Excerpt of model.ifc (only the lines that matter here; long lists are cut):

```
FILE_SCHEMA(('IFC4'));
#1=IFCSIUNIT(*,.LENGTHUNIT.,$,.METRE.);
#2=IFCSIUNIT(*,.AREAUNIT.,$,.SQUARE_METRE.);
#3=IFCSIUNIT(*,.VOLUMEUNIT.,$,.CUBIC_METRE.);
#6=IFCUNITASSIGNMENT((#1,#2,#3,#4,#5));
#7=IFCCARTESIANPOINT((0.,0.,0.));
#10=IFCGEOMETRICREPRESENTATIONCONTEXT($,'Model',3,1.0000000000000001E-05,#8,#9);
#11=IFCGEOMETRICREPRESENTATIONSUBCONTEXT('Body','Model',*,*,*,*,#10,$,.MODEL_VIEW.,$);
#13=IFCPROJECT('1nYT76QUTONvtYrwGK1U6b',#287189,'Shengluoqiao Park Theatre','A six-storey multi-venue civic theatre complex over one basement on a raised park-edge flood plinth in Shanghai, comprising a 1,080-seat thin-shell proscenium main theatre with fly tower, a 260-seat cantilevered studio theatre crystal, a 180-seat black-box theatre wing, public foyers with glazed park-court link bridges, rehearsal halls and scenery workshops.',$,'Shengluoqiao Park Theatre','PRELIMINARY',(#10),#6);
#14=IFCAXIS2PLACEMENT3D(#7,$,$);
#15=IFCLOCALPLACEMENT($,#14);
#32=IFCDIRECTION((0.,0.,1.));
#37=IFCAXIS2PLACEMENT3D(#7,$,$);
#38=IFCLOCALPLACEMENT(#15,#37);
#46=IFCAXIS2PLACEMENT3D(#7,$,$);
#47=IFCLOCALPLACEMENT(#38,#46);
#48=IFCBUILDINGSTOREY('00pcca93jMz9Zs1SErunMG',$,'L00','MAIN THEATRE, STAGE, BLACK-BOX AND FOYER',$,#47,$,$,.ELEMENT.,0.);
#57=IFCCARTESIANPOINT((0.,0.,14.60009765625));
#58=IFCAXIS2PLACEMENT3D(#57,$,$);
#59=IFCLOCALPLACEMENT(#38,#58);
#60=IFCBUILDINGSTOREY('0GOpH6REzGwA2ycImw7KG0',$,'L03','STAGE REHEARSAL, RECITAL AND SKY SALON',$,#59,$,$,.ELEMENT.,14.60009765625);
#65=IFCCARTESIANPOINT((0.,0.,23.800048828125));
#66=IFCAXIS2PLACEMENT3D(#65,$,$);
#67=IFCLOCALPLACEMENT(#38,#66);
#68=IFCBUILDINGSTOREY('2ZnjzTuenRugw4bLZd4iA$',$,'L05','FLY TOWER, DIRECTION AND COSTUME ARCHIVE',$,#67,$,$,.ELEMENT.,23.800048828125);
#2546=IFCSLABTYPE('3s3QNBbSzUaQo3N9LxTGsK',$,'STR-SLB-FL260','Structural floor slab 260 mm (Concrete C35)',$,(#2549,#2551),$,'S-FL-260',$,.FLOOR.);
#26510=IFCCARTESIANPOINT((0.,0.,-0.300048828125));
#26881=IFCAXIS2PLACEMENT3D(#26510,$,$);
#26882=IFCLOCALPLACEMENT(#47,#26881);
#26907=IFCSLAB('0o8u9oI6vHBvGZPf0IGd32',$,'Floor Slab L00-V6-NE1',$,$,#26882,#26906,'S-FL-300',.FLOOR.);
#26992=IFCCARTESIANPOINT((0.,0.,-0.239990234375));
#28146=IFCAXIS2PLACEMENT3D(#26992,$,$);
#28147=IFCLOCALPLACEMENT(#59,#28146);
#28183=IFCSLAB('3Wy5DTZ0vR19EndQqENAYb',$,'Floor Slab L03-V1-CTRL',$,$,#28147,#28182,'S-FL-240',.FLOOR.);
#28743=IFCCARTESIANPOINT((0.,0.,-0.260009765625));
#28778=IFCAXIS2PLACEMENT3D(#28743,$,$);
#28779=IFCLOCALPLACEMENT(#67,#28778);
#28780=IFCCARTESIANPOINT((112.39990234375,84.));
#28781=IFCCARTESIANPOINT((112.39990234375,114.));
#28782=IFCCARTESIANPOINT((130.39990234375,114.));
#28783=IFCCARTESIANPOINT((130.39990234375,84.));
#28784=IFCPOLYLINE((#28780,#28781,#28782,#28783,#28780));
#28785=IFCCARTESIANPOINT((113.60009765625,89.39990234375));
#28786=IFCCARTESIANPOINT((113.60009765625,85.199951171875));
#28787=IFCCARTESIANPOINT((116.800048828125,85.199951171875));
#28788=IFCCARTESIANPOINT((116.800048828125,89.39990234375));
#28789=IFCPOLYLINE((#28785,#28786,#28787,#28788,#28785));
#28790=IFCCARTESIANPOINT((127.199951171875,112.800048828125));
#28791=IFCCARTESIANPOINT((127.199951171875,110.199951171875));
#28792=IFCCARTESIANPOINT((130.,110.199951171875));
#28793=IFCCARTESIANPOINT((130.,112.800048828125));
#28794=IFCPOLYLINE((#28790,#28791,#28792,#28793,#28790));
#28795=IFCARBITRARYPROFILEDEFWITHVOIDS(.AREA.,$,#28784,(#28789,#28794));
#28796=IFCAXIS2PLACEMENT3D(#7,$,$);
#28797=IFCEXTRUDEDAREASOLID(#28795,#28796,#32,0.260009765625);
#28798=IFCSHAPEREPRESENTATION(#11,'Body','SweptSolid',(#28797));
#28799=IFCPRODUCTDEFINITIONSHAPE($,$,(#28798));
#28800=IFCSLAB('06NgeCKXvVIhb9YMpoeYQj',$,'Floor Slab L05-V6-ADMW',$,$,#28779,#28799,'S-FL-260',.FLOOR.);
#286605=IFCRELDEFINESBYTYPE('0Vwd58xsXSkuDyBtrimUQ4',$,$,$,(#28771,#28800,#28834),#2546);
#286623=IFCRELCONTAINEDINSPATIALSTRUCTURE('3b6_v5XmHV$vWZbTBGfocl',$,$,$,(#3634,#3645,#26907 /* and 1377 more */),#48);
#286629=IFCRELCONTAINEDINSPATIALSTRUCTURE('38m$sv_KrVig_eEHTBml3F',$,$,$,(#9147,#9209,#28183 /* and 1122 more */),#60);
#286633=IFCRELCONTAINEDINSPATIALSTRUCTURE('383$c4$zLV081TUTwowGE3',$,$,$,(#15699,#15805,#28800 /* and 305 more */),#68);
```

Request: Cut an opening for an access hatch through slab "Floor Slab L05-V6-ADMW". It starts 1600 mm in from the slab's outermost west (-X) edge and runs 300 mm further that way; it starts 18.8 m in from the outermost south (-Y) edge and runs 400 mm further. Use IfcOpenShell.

```python
import numpy as np
import ifcopenshell
import ifcopenshell.api.feature
import ifcopenshell.api.geometry
import ifcopenshell.api.root
import ifcopenshell.geom
import ifcopenshell.util.placement
import ifcopenshell.util.representation
import ifcopenshell.util.shape
import ifcopenshell.util.unit

model = ifcopenshell.open("model.ifc")
unit_scale = ifcopenshell.util.unit.calculate_unit_scale(model)
settings = ifcopenshell.geom.settings()


def volume(element):
    """Net volume in cubic metres, openings subtracted."""
    shape = ifcopenshell.geom.create_shape(settings, element)
    return ifcopenshell.util.shape.get_volume(shape.geometry)


slab = model.by_guid("06NgeCKXvVIhb9YMpoeYQj")
before = volume(slab)

# Extent in the slab's own axes, in metres. The edges named are its -X and -Y sides.
slab_shape = ifcopenshell.geom.create_shape(settings, slab)
vertices = ifcopenshell.util.shape.get_vertices(slab_shape.geometry)
x_min, y_min, bottom = vertices.min(axis=0)
top = vertices[:, 2].max()

opening = ifcopenshell.api.root.create_entity(model, ifc_class="IfcOpeningElement", name="Access hatch opening", predefined_type="OPENING")
context = ifcopenshell.util.representation.get_context(model, "Model", "Body", "MODEL_VIEW")
width, depth = 0.3, 0.4
outline = [(0.0, 0.0), (width, 0.0), (width, depth), (0.0, depth), (0.0, 0.0)]
# Overshoot both faces by 50 mm so the cut is clean.
shape = ifcopenshell.api.geometry.add_slab_representation(
    model, context=context, depth=top - bottom + 0.1, polyline=outline
)
ifcopenshell.api.geometry.assign_representation(model, product=opening, representation=shape)

matrix = ifcopenshell.util.placement.get_local_placement(slab.ObjectPlacement)
matrix[:, 3] = matrix @ np.append(np.array([x_min + 1.6, y_min + 18.8, bottom - 0.05]) / unit_scale, 1.0)
ifcopenshell.api.geometry.edit_object_placement(model, product=opening, matrix=matrix, is_si=False)
ifcopenshell.api.feature.add_feature(model, feature=opening, element=slab)

after = volume(slab)

print(f"slab volume {before:.3f} -> {after:.3f} m3")

model.write("model_rev.ifc")
```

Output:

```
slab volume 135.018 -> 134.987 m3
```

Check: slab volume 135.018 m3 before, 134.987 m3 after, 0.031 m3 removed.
